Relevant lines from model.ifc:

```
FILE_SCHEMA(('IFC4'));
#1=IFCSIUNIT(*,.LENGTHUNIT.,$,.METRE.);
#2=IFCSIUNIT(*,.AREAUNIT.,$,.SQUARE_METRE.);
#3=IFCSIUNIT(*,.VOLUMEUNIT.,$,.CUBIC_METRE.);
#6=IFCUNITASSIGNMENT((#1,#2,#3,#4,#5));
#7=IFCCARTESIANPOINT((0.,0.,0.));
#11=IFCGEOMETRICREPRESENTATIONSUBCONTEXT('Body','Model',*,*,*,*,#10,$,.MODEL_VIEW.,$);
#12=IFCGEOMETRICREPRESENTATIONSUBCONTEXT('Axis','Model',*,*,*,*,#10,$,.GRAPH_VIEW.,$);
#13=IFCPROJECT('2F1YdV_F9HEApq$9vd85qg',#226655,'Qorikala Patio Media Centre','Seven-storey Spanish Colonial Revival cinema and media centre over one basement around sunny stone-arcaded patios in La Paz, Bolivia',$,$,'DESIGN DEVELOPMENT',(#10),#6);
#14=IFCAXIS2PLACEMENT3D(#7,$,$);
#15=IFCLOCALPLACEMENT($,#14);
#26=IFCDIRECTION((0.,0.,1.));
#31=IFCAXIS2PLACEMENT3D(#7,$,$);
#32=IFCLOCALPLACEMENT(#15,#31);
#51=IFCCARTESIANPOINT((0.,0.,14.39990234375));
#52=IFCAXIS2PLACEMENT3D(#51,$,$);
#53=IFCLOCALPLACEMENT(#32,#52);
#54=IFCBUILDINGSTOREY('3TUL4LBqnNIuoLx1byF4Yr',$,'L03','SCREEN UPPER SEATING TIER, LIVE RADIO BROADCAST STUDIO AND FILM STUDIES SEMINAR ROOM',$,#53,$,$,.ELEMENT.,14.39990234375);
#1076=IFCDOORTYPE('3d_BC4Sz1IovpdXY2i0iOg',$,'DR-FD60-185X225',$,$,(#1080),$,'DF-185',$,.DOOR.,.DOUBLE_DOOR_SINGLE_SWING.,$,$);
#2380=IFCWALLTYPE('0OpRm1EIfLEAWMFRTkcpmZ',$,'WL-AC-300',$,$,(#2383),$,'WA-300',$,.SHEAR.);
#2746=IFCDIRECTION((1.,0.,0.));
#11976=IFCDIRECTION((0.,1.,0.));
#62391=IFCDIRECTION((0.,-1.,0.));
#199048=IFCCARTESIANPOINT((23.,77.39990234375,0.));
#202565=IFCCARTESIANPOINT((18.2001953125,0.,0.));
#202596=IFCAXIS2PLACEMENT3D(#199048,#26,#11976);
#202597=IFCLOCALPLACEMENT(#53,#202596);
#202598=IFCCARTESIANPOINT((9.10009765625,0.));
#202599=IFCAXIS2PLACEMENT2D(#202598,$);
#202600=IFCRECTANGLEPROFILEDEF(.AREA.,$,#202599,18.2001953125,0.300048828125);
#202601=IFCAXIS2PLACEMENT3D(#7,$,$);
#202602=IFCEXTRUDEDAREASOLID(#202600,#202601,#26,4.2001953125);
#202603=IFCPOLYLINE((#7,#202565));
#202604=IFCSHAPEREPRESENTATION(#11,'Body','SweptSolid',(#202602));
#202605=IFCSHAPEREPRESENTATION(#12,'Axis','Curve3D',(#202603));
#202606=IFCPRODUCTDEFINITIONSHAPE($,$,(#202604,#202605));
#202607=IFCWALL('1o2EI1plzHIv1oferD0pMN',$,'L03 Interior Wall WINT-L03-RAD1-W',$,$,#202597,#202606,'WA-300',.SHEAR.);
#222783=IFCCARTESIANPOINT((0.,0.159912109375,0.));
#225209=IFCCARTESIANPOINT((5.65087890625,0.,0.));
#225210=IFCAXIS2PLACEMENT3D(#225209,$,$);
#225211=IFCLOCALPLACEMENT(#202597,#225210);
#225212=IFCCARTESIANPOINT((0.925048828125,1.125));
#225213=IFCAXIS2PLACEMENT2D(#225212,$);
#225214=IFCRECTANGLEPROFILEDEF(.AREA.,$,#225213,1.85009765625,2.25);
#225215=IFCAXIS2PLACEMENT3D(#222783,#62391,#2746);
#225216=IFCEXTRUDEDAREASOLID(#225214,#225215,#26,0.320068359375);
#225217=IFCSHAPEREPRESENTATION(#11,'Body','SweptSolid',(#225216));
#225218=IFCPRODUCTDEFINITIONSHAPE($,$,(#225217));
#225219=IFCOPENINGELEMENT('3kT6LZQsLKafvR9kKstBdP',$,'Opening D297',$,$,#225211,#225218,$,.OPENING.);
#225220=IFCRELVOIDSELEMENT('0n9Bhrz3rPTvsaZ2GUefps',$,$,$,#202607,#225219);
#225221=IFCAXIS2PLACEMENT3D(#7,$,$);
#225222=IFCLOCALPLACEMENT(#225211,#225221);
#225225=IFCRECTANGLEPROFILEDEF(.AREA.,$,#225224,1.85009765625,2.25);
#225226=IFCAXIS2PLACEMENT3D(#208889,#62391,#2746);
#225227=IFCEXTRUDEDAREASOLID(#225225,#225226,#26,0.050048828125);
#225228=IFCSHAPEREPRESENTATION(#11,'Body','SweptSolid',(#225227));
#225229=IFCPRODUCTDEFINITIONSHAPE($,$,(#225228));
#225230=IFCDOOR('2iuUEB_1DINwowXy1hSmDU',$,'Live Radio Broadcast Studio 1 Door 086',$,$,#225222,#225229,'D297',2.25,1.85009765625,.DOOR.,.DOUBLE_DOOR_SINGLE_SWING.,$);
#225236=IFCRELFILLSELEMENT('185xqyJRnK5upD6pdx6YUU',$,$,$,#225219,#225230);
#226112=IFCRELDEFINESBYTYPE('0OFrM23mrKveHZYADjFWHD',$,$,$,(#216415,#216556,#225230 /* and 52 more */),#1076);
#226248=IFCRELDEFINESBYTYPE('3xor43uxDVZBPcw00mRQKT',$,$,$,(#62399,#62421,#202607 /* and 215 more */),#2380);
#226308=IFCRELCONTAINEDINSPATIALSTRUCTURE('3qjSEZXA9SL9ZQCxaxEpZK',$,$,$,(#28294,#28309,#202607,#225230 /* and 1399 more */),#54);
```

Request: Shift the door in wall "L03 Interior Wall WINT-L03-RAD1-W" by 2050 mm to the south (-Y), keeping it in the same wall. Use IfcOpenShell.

```python
import ifcopenshell
import ifcopenshell.api.geometry
import ifcopenshell.util.placement
import ifcopenshell.util.unit

model = ifcopenshell.open("model.ifc")
unit_scale = ifcopenshell.util.unit.calculate_unit_scale(model)

door = model.by_guid("2iuUEB_1DINwowXy1hSmDU")
opening = door.FillsVoids[0].RelatingOpeningElement
wall = opening.VoidsElements[0].RelatingBuildingElement

wall_matrix = ifcopenshell.util.placement.get_local_placement(wall.ObjectPlacement)
shift = wall_matrix[:3, 0] * -2.05 / unit_scale
before = ifcopenshell.util.placement.get_local_placement(door.ObjectPlacement)[:3, 3].copy()

# The door is placed relative to its opening, so it follows when the opening moves.
matrix = ifcopenshell.util.placement.get_local_placement(opening.ObjectPlacement)
matrix[:3, 3] += shift
ifcopenshell.api.geometry.edit_object_placement(
    model, product=opening, matrix=matrix, is_si=False, should_transform_children=True
)

after = ifcopenshell.util.placement.get_local_placement(door.ObjectPlacement)[:3, 3]
print("door moved by", (after - before).round(3) + 0.0)

model.write("model_rev.ifc")
```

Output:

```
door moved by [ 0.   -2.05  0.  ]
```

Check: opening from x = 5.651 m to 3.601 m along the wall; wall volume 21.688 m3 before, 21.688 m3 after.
